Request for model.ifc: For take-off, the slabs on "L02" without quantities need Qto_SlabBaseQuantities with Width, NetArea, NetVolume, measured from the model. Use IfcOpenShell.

First a look at what the model holds.

```python
import ifcopenshell
import ifcopenshell.util.element
import ifcopenshell.util.unit

model = ifcopenshell.open("model.ifc")
print(model.schema)
for unit_type in ("LENGTHUNIT", "AREAUNIT", "VOLUMEUNIT"):
    print(unit_type, ifcopenshell.util.unit.calculate_unit_scale(model, unit_type))
storey = next(s for s in model.by_type("IfcBuildingStorey") if s.Name == "L02")
slabs = [e for e in ifcopenshell.util.element.get_decomposition(storey) if e.is_a("IfcSlab")]
for e in sorted(slabs, key=lambda e: e.id()):
    print(e.id(), e.is_a(), e.Name, list(ifcopenshell.util.element.get_psets(e, qtos_only=True)), sep=" | ")
```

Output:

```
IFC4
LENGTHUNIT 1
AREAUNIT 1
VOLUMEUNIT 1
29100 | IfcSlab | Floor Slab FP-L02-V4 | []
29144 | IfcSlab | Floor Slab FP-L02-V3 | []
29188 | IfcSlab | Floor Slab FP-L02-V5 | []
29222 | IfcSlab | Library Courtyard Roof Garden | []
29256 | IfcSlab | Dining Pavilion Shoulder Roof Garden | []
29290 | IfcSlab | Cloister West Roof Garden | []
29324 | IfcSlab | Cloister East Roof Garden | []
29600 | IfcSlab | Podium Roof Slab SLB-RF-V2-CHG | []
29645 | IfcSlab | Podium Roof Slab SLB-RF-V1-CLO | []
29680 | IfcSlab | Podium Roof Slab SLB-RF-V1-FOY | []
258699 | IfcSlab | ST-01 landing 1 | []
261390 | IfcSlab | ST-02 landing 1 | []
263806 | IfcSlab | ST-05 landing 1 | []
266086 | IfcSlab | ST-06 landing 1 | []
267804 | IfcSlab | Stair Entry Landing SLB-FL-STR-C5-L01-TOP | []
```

```python
import ifcopenshell
import ifcopenshell.api.pset
import ifcopenshell.geom
import ifcopenshell.util.element
import ifcopenshell.util.shape
import ifcopenshell.util.unit

model = ifcopenshell.open("model.ifc")
unit_scale = ifcopenshell.util.unit.calculate_unit_scale(model)
area_scale = ifcopenshell.util.unit.calculate_unit_scale(model, "AREAUNIT")
volume_scale = ifcopenshell.util.unit.calculate_unit_scale(model, "VOLUMEUNIT")
settings = ifcopenshell.geom.settings()

storey = next(s for s in model.by_type("IfcBuildingStorey") if s.Name == "L02")
slabs = [e for e in ifcopenshell.util.element.get_decomposition(storey) if e.is_a("IfcSlab")]

for e in sorted(slabs, key=lambda e: e.id()):
    if ifcopenshell.util.element.get_psets(e, qtos_only=True, should_inherit=False):
        continue
    # Geometry comes back in metres, in the element's own axes.
    shape = ifcopenshell.geom.create_shape(settings, e)
    values = {
        "Width": ifcopenshell.util.shape.get_z(shape.geometry) / unit_scale,
        "NetArea": ifcopenshell.util.shape.get_footprint_area(shape.geometry) / area_scale,
        "NetVolume": ifcopenshell.util.shape.get_volume(shape.geometry) / volume_scale,
    }
    qto = ifcopenshell.api.pset.add_qto(model, product=e, name="Qto_SlabBaseQuantities")
    ifcopenshell.api.pset.edit_qto(model, qto=qto, properties=values)
    print(e.id(), {k: round(v, 3) for k, v in values.items()})

model.write("model_updated.ifc")
```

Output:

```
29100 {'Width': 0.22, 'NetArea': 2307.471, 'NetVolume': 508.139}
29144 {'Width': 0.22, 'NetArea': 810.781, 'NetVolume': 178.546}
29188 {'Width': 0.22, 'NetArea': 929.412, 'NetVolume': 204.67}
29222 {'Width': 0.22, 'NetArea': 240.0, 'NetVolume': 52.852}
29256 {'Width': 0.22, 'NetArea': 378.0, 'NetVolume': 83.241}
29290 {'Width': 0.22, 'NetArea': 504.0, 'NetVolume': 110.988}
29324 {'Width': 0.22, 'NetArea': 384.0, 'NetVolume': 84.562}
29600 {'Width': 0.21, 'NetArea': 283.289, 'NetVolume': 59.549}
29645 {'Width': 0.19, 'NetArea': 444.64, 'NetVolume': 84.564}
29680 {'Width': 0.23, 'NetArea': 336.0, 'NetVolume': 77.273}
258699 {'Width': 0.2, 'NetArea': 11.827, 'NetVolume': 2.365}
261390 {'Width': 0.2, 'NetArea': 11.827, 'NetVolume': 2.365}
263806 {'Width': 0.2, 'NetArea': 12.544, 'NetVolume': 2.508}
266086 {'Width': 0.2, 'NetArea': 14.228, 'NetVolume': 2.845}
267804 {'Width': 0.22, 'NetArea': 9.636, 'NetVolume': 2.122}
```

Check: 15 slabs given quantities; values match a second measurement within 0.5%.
